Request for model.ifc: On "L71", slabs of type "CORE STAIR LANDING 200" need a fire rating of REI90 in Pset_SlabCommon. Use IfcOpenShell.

First a look at what the model holds.

```python
import ifcopenshell
import ifcopenshell.util.element

model = ifcopenshell.open("model.ifc")
print(model.schema)
storey = next(s for s in model.by_type("IfcBuildingStorey") if s.Name == "L71")
slabs = [e for e in ifcopenshell.util.element.get_decomposition(storey) if e.is_a("IfcSlab")]
seen = {}
for e in slabs:
    element_type = ifcopenshell.util.element.get_type(e)
    key = (element_type.Name if element_type != e and element_type else None, ifcopenshell.util.element.get_pset(e, "Pset_SlabCommon", "FireRating"))
    seen[key] = seen.get(key, 0) + 1
for (name, value), count in sorted(seen.items(), key=str):
    print(count, "x", name, "|", value)
```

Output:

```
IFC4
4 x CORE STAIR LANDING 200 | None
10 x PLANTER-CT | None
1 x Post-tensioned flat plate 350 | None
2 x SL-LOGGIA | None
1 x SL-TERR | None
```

```python
import ifcopenshell
import ifcopenshell.api.pset
import ifcopenshell.util.element

model = ifcopenshell.open("model.ifc")

storey = next(s for s in model.by_type("IfcBuildingStorey") if s.Name == "L71")
slabs = [e for e in ifcopenshell.util.element.get_decomposition(storey) if e.is_a("IfcSlab")]

count = 0
for e in slabs:
    element_type = ifcopenshell.util.element.get_type(e)
    if element_type in (None, e) or element_type.Name != "CORE STAIR LANDING 200":
        continue
    found = ifcopenshell.util.element.get_pset(e, "Pset_SlabCommon", should_inherit=False)
    if found:
        pset = model.by_id(found["id"])
        if len(ifcopenshell.util.element.get_elements_by_pset(pset)) > 1:
            pset = ifcopenshell.api.pset.unshare_pset(model, products=[e], pset=pset)[0]
    else:
        pset = ifcopenshell.api.pset.add_pset(model, product=e, name="Pset_SlabCommon")
    ifcopenshell.api.pset.edit_pset(model, pset=pset, properties={"FireRating": "REI90"})
    count += 1

print(count, "slabs updated")

model.write("model_edited.ifc")
```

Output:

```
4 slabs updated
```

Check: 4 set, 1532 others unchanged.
